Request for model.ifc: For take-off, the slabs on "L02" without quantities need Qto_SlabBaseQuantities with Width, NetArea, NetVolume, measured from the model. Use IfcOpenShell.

First a look at what the model holds.

```python
import ifcopenshell
import ifcopenshell.util.element
import ifcopenshell.util.unit

model = ifcopenshell.open("model.ifc")
print(model.schema)
for unit_type in ("LENGTHUNIT", "AREAUNIT", "VOLUMEUNIT"):
    print(unit_type, ifcopenshell.util.unit.calculate_unit_scale(model, unit_type))
storey = next(s for s in model.by_type("IfcBuildingStorey") if s.Name == "L02")
slabs = [e for e in ifcopenshell.util.element.get_decomposition(storey) if e.is_a("IfcSlab")]
for e in sorted(slabs, key=lambda e: e.id()):
    print(e.id(), e.is_a(), e.Name, list(ifcopenshell.util.element.get_psets(e, qtos_only=True)), sep=" | ")
```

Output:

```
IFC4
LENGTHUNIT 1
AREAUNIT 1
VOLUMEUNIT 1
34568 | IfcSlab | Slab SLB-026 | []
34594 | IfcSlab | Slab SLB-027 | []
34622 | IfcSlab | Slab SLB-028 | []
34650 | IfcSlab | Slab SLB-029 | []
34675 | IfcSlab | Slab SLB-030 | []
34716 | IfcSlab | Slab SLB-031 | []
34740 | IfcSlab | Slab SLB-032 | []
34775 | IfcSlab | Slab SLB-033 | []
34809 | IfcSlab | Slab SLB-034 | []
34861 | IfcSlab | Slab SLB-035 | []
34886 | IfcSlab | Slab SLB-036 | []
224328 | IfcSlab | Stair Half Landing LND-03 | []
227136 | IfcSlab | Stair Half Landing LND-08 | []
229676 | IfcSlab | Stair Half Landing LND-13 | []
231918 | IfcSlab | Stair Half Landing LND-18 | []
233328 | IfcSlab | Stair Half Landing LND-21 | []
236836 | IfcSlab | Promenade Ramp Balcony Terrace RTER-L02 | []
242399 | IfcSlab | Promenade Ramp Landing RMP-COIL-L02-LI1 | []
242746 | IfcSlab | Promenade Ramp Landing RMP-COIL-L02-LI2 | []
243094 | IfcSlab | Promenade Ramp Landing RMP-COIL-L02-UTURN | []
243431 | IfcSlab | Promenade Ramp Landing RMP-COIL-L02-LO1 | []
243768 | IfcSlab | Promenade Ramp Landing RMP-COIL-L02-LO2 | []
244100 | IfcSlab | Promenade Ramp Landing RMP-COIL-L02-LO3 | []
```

```python
import ifcopenshell
import ifcopenshell.api.pset
import ifcopenshell.geom
import ifcopenshell.util.element
import ifcopenshell.util.shape
import ifcopenshell.util.unit

model = ifcopenshell.open("model.ifc")
unit_scale = ifcopenshell.util.unit.calculate_unit_scale(model)
area_scale = ifcopenshell.util.unit.calculate_unit_scale(model, "AREAUNIT")
volume_scale = ifcopenshell.util.unit.calculate_unit_scale(model, "VOLUMEUNIT")
settings = ifcopenshell.geom.settings()

storey = next(s for s in model.by_type("IfcBuildingStorey") if s.Name == "L02")
slabs = [e for e in ifcopenshell.util.element.get_decomposition(storey) if e.is_a("IfcSlab")]

for e in sorted(slabs, key=lambda e: e.id()):
    if ifcopenshell.util.element.get_psets(e, qtos_only=True, should_inherit=False):
        continue
    # Geometry comes back in metres, in the element's own axes.
    shape = ifcopenshell.geom.create_shape(settings, e)
    values = {
        "Width": ifcopenshell.util.shape.get_z(shape.geometry) / unit_scale,
        "NetArea": ifcopenshell.util.shape.get_footprint_area(shape.geometry) / area_scale,
        "NetVolume": ifcopenshell.util.shape.get_volume(shape.geometry) / volume_scale,
    }
    qto = ifcopenshell.api.pset.add_qto(model, product=e, name="Qto_SlabBaseQuantities")
    ifcopenshell.api.pset.edit_qto(model, qto=qto, properties=values)
    print(e.id(), {k: round(v, 3) for k, v in values.items()})

model.write("model_updated.ifc")
```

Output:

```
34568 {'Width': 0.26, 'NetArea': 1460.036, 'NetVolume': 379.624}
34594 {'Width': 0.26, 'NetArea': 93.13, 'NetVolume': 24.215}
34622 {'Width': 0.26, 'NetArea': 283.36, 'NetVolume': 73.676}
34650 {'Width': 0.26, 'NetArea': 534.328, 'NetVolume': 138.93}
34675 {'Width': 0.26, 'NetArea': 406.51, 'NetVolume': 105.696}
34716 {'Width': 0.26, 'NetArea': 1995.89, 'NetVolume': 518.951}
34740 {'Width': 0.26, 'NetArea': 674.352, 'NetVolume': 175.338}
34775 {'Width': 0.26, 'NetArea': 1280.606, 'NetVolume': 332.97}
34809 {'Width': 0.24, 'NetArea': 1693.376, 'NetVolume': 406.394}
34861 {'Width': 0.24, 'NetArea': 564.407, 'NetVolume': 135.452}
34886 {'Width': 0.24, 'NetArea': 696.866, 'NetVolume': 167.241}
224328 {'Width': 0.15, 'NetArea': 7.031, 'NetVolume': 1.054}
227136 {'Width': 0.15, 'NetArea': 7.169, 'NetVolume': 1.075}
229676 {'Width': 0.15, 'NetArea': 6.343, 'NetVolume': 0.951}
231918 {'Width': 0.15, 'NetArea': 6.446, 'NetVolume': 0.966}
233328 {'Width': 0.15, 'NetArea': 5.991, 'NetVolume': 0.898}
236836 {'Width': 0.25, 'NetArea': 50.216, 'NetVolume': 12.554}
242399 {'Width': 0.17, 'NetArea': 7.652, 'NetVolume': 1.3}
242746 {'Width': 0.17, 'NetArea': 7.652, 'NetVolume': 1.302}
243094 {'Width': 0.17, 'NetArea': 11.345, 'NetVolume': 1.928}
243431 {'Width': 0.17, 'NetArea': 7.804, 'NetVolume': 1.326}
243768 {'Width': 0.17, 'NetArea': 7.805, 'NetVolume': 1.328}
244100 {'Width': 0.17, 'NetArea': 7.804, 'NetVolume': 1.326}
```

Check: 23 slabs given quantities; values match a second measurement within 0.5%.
